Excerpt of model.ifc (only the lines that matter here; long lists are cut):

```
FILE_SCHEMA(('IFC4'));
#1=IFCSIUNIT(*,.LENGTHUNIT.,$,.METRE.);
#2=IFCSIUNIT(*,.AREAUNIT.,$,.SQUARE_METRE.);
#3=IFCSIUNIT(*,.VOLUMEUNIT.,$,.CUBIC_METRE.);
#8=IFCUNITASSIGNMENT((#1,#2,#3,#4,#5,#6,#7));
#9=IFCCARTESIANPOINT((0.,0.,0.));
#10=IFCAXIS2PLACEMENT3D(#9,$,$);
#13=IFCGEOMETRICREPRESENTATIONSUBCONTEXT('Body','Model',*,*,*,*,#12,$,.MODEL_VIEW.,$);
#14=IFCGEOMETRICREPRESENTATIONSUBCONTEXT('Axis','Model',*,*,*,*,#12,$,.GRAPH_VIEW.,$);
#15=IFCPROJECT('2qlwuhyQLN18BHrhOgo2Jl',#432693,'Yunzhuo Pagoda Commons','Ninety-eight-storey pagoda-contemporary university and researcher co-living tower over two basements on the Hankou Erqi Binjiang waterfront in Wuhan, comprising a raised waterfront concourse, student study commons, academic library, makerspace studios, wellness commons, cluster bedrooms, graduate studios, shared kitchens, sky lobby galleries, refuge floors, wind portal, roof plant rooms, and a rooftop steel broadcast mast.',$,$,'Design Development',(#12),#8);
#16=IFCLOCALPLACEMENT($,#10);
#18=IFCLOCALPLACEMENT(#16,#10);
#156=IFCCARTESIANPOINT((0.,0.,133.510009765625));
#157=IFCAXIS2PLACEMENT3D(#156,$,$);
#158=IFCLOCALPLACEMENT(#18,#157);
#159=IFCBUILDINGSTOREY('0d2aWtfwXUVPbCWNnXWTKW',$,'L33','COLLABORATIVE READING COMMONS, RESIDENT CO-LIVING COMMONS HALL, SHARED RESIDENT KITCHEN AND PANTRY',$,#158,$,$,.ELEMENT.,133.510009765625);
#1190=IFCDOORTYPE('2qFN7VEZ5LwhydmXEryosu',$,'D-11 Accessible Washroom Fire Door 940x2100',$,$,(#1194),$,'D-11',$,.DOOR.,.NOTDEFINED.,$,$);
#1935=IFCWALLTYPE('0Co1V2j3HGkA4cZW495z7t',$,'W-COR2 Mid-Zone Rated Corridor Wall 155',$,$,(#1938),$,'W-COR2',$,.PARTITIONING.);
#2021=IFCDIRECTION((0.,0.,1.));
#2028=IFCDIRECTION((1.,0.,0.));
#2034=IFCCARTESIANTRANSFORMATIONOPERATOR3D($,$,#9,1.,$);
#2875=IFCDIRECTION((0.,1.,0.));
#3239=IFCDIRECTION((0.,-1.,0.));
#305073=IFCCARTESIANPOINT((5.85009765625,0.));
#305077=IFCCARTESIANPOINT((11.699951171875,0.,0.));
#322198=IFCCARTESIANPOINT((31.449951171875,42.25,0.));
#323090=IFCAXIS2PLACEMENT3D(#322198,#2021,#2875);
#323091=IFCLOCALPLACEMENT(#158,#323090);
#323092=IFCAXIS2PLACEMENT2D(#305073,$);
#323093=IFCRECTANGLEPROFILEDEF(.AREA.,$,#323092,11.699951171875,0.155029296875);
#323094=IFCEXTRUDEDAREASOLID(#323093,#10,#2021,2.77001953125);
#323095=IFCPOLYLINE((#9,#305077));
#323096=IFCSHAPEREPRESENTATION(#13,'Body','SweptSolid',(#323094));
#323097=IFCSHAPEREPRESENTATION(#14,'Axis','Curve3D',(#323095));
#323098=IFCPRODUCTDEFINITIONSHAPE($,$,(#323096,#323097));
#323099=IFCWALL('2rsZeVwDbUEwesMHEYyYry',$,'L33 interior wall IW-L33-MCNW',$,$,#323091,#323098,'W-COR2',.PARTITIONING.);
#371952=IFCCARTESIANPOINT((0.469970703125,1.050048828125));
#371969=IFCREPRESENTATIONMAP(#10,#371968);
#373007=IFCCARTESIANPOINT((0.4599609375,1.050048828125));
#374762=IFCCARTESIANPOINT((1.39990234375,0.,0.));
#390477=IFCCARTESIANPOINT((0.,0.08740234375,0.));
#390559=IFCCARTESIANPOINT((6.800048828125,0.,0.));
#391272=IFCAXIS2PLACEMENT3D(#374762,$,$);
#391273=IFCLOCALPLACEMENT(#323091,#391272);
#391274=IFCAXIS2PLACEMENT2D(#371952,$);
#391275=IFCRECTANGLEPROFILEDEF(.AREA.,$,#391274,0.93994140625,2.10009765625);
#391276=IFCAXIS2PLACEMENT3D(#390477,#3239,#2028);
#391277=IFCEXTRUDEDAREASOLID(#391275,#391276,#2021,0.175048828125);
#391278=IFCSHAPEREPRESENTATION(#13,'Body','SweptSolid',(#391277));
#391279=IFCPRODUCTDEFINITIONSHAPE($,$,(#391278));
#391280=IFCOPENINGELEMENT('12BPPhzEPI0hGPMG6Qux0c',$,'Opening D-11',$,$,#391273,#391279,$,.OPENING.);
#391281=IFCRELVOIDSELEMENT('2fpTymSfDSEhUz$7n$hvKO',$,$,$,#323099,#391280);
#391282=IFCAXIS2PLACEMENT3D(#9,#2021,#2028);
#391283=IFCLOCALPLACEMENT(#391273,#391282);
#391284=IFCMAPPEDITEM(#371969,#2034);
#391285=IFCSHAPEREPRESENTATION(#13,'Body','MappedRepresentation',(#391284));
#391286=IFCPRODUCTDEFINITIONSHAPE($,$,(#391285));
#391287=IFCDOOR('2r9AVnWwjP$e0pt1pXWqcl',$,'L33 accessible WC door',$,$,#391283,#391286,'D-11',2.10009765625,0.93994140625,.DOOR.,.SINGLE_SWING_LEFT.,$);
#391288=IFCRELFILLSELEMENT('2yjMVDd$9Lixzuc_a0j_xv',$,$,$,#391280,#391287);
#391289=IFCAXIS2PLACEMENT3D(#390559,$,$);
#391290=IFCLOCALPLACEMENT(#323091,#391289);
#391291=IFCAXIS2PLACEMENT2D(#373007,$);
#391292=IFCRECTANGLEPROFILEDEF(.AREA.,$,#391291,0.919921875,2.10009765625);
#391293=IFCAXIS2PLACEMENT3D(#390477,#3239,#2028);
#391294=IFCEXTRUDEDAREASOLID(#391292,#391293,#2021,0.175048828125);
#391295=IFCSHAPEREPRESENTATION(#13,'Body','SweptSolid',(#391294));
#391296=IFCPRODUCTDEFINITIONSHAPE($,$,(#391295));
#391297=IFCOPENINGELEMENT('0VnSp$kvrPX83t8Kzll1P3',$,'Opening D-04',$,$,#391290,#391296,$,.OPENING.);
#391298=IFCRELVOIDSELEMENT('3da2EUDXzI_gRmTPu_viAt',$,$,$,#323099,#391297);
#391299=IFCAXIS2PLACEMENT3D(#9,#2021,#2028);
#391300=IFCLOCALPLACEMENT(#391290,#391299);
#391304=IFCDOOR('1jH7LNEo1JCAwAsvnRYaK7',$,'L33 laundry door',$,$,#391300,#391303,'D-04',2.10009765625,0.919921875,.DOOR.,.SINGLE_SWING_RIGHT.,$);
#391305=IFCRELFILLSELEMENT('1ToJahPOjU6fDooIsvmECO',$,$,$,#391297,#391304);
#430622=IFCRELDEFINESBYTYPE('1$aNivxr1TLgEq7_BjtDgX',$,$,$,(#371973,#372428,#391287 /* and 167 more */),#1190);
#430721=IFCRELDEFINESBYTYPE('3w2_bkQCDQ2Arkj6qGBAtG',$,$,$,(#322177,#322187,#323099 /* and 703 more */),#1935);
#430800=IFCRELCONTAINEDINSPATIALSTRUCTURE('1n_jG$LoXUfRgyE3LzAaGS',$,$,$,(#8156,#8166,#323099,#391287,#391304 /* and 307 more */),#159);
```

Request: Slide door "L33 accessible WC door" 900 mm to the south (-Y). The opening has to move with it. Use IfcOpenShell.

```python
import ifcopenshell
import ifcopenshell.api.geometry
import ifcopenshell.util.placement
import ifcopenshell.util.unit

model = ifcopenshell.open("model.ifc")
unit_scale = ifcopenshell.util.unit.calculate_unit_scale(model)

door = model.by_guid("2r9AVnWwjP$e0pt1pXWqcl")
opening = door.FillsVoids[0].RelatingOpeningElement
wall = opening.VoidsElements[0].RelatingBuildingElement

wall_matrix = ifcopenshell.util.placement.get_local_placement(wall.ObjectPlacement)
shift = wall_matrix[:3, 0] * -0.9 / unit_scale
before = ifcopenshell.util.placement.get_local_placement(door.ObjectPlacement)[:3, 3].copy()

# The door is placed relative to its opening, so it follows when the opening moves.
matrix = ifcopenshell.util.placement.get_local_placement(opening.ObjectPlacement)
matrix[:3, 3] += shift
ifcopenshell.api.geometry.edit_object_placement(
    model, product=opening, matrix=matrix, is_si=False, should_transform_children=True
)

after = ifcopenshell.util.placement.get_local_placement(door.ObjectPlacement)[:3, 3]
print("door moved by", (after - before).round(3) + 0.0)

model.write("model_v2.ifc")
```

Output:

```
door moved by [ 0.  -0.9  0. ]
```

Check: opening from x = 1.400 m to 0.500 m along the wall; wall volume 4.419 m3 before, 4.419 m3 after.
